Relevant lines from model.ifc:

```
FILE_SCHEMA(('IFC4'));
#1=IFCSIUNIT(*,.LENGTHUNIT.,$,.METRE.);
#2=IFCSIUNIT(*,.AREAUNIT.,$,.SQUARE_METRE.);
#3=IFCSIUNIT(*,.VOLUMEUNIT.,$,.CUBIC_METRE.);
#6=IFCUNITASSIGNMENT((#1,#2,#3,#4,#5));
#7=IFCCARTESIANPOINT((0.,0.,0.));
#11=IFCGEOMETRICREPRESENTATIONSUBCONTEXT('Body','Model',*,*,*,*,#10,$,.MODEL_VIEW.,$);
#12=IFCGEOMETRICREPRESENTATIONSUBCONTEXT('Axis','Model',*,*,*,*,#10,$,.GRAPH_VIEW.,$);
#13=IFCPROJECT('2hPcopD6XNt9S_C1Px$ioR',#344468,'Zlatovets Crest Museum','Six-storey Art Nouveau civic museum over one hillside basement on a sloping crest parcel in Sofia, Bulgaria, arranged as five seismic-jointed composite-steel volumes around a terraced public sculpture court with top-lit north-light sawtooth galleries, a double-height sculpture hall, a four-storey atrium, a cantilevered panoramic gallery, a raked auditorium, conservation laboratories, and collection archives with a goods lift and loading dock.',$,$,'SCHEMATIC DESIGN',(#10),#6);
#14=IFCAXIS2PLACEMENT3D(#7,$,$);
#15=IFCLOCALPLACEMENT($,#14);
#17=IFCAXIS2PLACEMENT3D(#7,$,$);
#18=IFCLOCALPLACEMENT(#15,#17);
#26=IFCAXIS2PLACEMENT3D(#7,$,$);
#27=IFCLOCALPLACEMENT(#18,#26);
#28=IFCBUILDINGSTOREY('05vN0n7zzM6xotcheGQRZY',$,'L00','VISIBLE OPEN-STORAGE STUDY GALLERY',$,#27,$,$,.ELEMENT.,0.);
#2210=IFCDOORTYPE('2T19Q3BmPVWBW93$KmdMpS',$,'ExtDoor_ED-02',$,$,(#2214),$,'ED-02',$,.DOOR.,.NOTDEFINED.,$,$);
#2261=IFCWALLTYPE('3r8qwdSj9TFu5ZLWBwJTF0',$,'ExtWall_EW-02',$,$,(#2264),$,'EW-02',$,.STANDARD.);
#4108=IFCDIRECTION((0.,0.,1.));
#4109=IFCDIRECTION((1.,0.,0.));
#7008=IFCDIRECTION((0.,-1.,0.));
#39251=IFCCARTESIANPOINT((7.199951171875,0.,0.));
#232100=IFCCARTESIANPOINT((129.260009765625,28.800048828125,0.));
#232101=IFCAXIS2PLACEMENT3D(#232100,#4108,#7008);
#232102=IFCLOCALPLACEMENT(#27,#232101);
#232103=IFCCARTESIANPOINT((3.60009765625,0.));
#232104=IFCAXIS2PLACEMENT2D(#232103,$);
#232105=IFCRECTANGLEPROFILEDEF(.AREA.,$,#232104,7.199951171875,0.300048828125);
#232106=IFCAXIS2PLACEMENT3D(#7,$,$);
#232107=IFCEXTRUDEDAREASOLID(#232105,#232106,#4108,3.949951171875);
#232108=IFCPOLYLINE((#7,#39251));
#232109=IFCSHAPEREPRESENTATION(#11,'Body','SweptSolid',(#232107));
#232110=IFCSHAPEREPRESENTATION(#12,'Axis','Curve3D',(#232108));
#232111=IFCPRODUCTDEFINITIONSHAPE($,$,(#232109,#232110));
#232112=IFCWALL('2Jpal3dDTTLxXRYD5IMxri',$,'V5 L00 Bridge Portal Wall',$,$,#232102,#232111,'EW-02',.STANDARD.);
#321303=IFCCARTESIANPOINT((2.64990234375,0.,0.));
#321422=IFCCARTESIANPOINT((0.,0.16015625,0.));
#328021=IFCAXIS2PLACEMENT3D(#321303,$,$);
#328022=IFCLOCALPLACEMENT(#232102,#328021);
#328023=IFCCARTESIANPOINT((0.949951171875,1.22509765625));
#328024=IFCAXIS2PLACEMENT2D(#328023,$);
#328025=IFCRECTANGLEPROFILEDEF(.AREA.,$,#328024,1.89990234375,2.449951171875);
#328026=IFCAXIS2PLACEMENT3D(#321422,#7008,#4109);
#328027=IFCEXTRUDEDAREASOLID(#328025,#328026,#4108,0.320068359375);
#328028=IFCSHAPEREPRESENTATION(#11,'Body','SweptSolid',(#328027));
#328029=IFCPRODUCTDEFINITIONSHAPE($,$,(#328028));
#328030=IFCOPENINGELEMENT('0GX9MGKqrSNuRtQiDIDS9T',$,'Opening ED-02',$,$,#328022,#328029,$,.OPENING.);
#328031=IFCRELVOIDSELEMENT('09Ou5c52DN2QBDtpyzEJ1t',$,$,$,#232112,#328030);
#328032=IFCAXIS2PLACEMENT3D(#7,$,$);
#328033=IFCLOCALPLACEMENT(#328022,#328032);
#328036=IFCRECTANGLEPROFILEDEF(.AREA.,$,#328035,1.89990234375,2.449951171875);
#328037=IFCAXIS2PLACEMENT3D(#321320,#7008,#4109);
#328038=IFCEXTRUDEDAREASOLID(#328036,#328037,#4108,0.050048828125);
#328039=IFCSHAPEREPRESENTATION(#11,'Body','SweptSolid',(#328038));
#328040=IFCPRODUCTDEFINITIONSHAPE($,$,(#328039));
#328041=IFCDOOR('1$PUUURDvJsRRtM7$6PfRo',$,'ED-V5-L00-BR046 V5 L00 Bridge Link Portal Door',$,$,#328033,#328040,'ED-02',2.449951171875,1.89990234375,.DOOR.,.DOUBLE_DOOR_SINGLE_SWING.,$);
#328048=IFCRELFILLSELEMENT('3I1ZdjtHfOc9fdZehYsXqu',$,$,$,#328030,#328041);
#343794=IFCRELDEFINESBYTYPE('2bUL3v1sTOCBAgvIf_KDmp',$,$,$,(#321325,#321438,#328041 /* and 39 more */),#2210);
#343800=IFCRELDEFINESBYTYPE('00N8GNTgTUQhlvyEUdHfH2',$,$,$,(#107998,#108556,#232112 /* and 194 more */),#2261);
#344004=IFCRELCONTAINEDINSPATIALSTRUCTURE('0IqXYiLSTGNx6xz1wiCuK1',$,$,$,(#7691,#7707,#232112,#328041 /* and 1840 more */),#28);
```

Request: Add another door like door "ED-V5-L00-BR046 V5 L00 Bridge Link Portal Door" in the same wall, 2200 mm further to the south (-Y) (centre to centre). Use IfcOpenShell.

```python
import ifcopenshell
import ifcopenshell.api.feature
import ifcopenshell.api.geometry
import ifcopenshell.api.root
import ifcopenshell.geom
import ifcopenshell.util.element
import ifcopenshell.util.placement
import ifcopenshell.util.shape
import ifcopenshell.util.unit

model = ifcopenshell.open("model.ifc")
unit_scale = ifcopenshell.util.unit.calculate_unit_scale(model)
settings = ifcopenshell.geom.settings()


def volume(element):
    """Net volume in cubic metres, openings subtracted."""
    shape = ifcopenshell.geom.create_shape(settings, element)
    return ifcopenshell.util.shape.get_volume(shape.geometry)


door = model.by_id(328041)
opening = door.FillsVoids[0].RelatingOpeningElement
wall = opening.VoidsElements[0].RelatingBuildingElement
before = volume(wall)
shift = ifcopenshell.util.placement.get_local_placement(wall.ObjectPlacement)[:3, 0] * 2.2 / unit_scale

# copy_class copies the void relationship, type, container and properties, but no geometry.
new_opening = ifcopenshell.api.root.copy_class(model, product=opening)
new_opening.Representation = ifcopenshell.util.element.copy_deep(
    model, opening.Representation, exclude=["IfcGeometricRepresentationContext", "IfcRepresentationMap"]
)
new_door = ifcopenshell.api.root.copy_class(model, product=door)
new_door.Representation = ifcopenshell.util.element.copy_deep(
    model, door.Representation, exclude=["IfcGeometricRepresentationContext", "IfcRepresentationMap"]
)
new_door.Tag = None
ifcopenshell.api.feature.add_filling(model, opening=new_opening, element=new_door)

for old, new in ((opening, new_opening), (door, new_door)):
    matrix = ifcopenshell.util.placement.get_local_placement(old.ObjectPlacement)
    matrix[:3, 3] += shift
    ifcopenshell.api.geometry.edit_object_placement(model, product=new, matrix=matrix, is_si=False)

after = volume(wall)

print(f"wall volume {before:.3f} -> {after:.3f} m3")

model.write("model-out.ifc")
```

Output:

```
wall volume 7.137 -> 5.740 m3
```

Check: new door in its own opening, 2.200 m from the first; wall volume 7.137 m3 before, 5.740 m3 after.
